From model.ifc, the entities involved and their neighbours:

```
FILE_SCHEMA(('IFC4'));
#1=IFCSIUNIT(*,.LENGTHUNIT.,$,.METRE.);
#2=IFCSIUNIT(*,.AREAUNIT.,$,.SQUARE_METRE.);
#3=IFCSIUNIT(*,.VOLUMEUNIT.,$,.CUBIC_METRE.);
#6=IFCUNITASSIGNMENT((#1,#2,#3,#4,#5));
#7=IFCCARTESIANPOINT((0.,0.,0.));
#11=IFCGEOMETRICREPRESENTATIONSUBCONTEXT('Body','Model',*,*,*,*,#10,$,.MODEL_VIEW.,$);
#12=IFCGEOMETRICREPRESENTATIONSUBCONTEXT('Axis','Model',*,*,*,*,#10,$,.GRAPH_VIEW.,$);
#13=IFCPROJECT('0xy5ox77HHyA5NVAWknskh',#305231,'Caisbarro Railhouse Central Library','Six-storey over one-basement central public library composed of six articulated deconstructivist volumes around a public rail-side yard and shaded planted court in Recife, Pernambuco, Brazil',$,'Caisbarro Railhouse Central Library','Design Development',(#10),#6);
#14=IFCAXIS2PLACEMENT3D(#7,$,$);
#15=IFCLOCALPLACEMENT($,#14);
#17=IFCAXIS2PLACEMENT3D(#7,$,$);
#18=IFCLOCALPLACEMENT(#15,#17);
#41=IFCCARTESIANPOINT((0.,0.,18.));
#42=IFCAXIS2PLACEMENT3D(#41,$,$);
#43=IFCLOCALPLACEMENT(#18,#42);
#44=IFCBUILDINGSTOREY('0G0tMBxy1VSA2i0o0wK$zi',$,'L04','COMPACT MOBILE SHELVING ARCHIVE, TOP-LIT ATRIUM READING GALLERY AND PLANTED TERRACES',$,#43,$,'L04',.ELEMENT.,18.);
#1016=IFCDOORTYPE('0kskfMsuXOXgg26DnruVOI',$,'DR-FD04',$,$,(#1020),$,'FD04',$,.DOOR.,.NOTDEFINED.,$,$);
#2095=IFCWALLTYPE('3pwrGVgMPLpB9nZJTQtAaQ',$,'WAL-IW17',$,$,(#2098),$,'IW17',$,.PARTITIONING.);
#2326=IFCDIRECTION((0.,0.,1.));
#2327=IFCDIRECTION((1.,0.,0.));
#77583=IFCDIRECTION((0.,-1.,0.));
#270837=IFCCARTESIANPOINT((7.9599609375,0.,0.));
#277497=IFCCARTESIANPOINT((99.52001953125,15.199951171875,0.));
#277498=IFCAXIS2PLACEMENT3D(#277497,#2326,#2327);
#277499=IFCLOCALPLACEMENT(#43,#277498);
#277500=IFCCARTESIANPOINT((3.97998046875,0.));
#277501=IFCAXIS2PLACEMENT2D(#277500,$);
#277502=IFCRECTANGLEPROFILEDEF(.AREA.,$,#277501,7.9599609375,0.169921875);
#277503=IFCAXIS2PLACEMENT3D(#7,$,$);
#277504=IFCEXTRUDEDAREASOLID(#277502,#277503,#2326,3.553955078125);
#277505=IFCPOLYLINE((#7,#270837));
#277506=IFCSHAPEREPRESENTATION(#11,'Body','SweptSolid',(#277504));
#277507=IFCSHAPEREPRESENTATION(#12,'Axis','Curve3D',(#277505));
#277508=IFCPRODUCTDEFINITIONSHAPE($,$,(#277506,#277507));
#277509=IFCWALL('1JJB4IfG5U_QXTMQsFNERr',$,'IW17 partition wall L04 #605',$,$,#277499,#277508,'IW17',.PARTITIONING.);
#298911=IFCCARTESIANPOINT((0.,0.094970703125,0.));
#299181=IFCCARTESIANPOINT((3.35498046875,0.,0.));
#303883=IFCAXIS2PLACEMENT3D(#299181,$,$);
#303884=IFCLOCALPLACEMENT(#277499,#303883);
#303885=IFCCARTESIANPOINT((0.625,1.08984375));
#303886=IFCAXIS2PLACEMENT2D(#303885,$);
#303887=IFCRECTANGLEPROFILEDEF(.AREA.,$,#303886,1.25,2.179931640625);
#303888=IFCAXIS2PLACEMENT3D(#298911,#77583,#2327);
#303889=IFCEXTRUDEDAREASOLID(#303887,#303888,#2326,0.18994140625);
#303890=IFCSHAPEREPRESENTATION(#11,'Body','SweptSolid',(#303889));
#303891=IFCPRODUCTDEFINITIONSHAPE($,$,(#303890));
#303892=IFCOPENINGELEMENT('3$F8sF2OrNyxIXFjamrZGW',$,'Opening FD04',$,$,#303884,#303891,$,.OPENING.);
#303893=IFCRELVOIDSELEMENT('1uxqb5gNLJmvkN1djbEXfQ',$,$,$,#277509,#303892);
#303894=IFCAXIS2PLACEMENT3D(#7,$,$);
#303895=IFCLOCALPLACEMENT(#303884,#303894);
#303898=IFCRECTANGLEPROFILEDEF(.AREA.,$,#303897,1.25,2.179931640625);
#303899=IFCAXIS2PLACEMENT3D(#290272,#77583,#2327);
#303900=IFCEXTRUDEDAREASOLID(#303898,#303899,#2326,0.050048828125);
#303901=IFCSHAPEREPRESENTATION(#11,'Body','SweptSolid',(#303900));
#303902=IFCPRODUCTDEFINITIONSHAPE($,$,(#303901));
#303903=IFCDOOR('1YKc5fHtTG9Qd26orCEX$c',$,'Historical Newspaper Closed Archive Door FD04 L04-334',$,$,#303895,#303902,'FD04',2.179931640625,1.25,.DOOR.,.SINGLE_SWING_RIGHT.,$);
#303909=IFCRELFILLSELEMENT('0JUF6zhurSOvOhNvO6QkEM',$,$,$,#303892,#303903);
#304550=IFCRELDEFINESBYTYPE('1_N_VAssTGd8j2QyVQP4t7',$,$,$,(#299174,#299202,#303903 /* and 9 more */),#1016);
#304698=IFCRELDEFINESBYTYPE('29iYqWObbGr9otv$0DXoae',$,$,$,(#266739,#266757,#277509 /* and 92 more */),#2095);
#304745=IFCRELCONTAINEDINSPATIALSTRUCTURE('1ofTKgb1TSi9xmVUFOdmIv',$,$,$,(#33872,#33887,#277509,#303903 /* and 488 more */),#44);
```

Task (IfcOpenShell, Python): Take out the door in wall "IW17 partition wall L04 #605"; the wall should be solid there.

```python
import ifcopenshell
import ifcopenshell.api.feature
import ifcopenshell.api.root
import ifcopenshell.geom
import ifcopenshell.util.shape

model = ifcopenshell.open("model.ifc")
settings = ifcopenshell.geom.settings()


def volume(element):
    """Net volume in cubic metres, openings subtracted."""
    shape = ifcopenshell.geom.create_shape(settings, element)
    return ifcopenshell.util.shape.get_volume(shape.geometry)


door = model.by_id(303903)
opening = door.FillsVoids[0].RelatingOpeningElement
wall = opening.VoidsElements[0].RelatingBuildingElement
before = volume(wall)

ifcopenshell.api.root.remove_product(model, product=door)
ifcopenshell.api.feature.remove_feature(model, feature=opening)

after = volume(wall)

print(f"wall volume {before:.3f} -> {after:.3f} m3")

model.write("model-out.ifc")
```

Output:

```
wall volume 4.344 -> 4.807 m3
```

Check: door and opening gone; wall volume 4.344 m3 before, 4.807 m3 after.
